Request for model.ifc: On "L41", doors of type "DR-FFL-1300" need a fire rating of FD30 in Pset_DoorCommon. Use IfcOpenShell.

First a look at what the model holds.

```python
import ifcopenshell
import ifcopenshell.util.element

model = ifcopenshell.open("model.ifc")
print(model.schema)
storey = next(s for s in model.by_type("IfcBuildingStorey") if s.Name == "L41")
doors = [e for e in ifcopenshell.util.element.get_decomposition(storey) if e.is_a("IfcDoor")]
seen = {}
for e in doors:
    element_type = ifcopenshell.util.element.get_type(e)
    key = (element_type.Name if element_type != e and element_type else None, ifcopenshell.util.element.get_pset(e, "Pset_DoorCommon", "FireRating"))
    seen[key] = seen.get(key, 0) + 1
for (name, value), count in sorted(seen.items(), key=str):
    print(count, "x", name, "|", value)
```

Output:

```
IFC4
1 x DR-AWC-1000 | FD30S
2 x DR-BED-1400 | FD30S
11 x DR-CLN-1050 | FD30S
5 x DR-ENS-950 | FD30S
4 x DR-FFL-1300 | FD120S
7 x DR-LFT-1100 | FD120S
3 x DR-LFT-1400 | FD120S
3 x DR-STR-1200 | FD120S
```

```python
import ifcopenshell
import ifcopenshell.api.pset
import ifcopenshell.util.element

model = ifcopenshell.open("model.ifc")

storey = next(s for s in model.by_type("IfcBuildingStorey") if s.Name == "L41")
doors = [e for e in ifcopenshell.util.element.get_decomposition(storey) if e.is_a("IfcDoor")]

count = 0
for e in doors:
    element_type = ifcopenshell.util.element.get_type(e)
    if element_type in (None, e) or element_type.Name != "DR-FFL-1300":
        continue
    # add_pset returns the element's existing set when there is one.
    pset = ifcopenshell.api.pset.add_pset(model, product=e, name="Pset_DoorCommon")
    ifcopenshell.api.pset.edit_pset(model, pset=pset, properties={"FireRating": "FD30"})
    count += 1

print(count, "doors updated")

model.write("model_rev.ifc")
```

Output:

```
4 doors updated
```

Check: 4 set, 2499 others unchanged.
